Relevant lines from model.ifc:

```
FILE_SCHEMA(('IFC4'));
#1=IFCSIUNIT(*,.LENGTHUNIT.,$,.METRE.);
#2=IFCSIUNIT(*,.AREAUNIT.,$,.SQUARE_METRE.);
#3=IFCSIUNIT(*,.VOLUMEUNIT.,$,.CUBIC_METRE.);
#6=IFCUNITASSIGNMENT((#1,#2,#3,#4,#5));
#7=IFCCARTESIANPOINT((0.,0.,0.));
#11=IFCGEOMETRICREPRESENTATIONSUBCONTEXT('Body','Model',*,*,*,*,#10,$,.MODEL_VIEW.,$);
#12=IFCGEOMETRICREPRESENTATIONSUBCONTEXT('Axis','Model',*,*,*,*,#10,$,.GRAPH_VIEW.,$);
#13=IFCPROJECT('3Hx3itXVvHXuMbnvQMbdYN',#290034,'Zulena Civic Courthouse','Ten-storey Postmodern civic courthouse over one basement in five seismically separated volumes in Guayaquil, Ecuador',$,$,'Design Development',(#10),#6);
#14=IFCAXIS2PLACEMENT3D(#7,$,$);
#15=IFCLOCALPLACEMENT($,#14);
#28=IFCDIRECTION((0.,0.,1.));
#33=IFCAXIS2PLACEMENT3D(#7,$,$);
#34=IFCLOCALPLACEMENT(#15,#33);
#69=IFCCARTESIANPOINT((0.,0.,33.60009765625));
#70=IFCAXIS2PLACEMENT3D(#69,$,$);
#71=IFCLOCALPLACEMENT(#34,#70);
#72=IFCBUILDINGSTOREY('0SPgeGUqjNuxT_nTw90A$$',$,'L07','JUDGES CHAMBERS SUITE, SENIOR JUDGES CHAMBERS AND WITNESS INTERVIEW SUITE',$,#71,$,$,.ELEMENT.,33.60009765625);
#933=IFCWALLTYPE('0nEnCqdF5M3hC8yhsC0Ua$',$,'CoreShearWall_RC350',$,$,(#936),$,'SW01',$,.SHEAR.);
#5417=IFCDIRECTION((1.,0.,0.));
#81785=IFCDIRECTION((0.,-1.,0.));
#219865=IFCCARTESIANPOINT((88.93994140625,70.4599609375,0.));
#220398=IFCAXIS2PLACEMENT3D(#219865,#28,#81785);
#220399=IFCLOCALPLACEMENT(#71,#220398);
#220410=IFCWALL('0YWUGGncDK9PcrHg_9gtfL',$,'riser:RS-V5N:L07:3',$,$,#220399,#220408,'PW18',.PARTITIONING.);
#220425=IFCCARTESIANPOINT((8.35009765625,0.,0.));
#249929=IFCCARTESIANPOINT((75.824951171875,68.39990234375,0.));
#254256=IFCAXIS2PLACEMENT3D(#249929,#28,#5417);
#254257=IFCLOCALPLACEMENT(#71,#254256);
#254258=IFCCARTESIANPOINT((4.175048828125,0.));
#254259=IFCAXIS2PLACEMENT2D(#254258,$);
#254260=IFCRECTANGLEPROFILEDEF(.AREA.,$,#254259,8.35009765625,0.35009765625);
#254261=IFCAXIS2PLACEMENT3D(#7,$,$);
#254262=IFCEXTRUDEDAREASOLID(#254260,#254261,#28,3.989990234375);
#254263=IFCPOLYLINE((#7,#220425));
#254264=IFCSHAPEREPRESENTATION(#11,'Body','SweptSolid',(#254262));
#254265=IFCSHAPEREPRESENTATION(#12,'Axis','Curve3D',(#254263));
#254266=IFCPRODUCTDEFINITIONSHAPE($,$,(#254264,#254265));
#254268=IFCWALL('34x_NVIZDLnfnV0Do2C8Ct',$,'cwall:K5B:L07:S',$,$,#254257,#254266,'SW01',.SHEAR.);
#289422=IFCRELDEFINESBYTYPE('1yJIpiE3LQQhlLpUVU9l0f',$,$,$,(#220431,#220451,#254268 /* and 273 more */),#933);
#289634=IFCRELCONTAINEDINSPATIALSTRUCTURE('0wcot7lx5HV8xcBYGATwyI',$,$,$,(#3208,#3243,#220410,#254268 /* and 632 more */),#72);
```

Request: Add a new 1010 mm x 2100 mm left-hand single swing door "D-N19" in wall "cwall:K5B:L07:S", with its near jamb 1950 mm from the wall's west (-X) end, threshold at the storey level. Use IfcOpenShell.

```python
import numpy as np
import ifcopenshell
import ifcopenshell.api.feature
import ifcopenshell.api.geometry
import ifcopenshell.api.root
import ifcopenshell.api.spatial
import ifcopenshell.geom
import ifcopenshell.util.element
import ifcopenshell.util.placement
import ifcopenshell.util.representation
import ifcopenshell.util.shape
import ifcopenshell.util.unit

model = ifcopenshell.open("model.ifc")
unit_scale = ifcopenshell.util.unit.calculate_unit_scale(model)
settings = ifcopenshell.geom.settings()


def volume(element):
    """Net volume in cubic metres, openings subtracted."""
    shape = ifcopenshell.geom.create_shape(settings, element)
    return ifcopenshell.util.shape.get_volume(shape.geometry)


wall = model.by_guid("34x_NVIZDLnfnV0Do2C8Ct")
storey = ifcopenshell.util.element.get_container(wall, ifc_class="IfcBuildingStorey")
context = ifcopenshell.util.representation.get_context(model, "Model", "Body", "MODEL_VIEW")
before = volume(wall)

width, height, from_end, sill = 1.01, 2.1, 1.95, 0.0  # metres

# The wall runs along its own X axis, and the end named is its -X end.
wall_shape = ifcopenshell.geom.create_shape(settings, wall)
x, y, z = ifcopenshell.util.shape.get_vertices(wall_shape.geometry).T
start = x.min() + from_end
face, thickness = float(y.min()), float(y.max() - y.min())
wall_matrix = ifcopenshell.util.placement.get_local_placement(wall.ObjectPlacement)
level = ifcopenshell.util.placement.get_local_placement(storey.ObjectPlacement)[2, 3]


def in_wall(x, y):
    """Placement at x, y metres in the wall's axes, at sill height."""
    matrix = wall_matrix.copy()
    matrix[:, 3] = wall_matrix @ np.array([x / unit_scale, y / unit_scale, 0.0, 1.0])
    matrix[2, 3] = level + sill / unit_scale
    return matrix


# Opening: a box that overshoots both wall faces by 50 mm.
opening = ifcopenshell.api.root.create_entity(model, ifc_class="IfcOpeningElement", predefined_type="OPENING")
box = ifcopenshell.api.geometry.add_wall_representation(
    model, context=context, length=width, height=height, thickness=thickness + 0.1
)
ifcopenshell.api.geometry.assign_representation(model, product=opening, representation=box)
ifcopenshell.api.geometry.edit_object_placement(model, product=opening, matrix=in_wall(start, face - 0.05), is_si=False)
ifcopenshell.api.feature.add_feature(model, feature=opening, element=wall)

door = ifcopenshell.api.root.create_entity(model, ifc_class="IfcDoor", name="D-N19", predefined_type="DOOR")
door.OverallWidth, door.OverallHeight = width / unit_scale, height / unit_scale
door.OperationType = "SINGLE_SWING_LEFT"
body = ifcopenshell.api.geometry.add_door_representation(
    model,
    context=context,
    overall_width=door.OverallWidth,
    overall_height=door.OverallHeight,
    operation_type="SINGLE_SWING_LEFT",
    lining_properties={"LiningDepth": thickness / unit_scale, "ThresholdDepth": thickness / unit_scale},
)
ifcopenshell.api.geometry.assign_representation(model, product=door, representation=body)
ifcopenshell.api.spatial.assign_container(model, products=[door], relating_structure=storey)
ifcopenshell.api.feature.add_filling(model, opening=opening, element=door)

# The lining spans the wall, so the door starts at the wall face.
ifcopenshell.api.geometry.edit_object_placement(model, product=door, matrix=in_wall(start, face), is_si=False)

after = volume(wall)

print(f"wall volume {before:.3f} -> {after:.3f} m3")

model.write("model_rev.ifc")
```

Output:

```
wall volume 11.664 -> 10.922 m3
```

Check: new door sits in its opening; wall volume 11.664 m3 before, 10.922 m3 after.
